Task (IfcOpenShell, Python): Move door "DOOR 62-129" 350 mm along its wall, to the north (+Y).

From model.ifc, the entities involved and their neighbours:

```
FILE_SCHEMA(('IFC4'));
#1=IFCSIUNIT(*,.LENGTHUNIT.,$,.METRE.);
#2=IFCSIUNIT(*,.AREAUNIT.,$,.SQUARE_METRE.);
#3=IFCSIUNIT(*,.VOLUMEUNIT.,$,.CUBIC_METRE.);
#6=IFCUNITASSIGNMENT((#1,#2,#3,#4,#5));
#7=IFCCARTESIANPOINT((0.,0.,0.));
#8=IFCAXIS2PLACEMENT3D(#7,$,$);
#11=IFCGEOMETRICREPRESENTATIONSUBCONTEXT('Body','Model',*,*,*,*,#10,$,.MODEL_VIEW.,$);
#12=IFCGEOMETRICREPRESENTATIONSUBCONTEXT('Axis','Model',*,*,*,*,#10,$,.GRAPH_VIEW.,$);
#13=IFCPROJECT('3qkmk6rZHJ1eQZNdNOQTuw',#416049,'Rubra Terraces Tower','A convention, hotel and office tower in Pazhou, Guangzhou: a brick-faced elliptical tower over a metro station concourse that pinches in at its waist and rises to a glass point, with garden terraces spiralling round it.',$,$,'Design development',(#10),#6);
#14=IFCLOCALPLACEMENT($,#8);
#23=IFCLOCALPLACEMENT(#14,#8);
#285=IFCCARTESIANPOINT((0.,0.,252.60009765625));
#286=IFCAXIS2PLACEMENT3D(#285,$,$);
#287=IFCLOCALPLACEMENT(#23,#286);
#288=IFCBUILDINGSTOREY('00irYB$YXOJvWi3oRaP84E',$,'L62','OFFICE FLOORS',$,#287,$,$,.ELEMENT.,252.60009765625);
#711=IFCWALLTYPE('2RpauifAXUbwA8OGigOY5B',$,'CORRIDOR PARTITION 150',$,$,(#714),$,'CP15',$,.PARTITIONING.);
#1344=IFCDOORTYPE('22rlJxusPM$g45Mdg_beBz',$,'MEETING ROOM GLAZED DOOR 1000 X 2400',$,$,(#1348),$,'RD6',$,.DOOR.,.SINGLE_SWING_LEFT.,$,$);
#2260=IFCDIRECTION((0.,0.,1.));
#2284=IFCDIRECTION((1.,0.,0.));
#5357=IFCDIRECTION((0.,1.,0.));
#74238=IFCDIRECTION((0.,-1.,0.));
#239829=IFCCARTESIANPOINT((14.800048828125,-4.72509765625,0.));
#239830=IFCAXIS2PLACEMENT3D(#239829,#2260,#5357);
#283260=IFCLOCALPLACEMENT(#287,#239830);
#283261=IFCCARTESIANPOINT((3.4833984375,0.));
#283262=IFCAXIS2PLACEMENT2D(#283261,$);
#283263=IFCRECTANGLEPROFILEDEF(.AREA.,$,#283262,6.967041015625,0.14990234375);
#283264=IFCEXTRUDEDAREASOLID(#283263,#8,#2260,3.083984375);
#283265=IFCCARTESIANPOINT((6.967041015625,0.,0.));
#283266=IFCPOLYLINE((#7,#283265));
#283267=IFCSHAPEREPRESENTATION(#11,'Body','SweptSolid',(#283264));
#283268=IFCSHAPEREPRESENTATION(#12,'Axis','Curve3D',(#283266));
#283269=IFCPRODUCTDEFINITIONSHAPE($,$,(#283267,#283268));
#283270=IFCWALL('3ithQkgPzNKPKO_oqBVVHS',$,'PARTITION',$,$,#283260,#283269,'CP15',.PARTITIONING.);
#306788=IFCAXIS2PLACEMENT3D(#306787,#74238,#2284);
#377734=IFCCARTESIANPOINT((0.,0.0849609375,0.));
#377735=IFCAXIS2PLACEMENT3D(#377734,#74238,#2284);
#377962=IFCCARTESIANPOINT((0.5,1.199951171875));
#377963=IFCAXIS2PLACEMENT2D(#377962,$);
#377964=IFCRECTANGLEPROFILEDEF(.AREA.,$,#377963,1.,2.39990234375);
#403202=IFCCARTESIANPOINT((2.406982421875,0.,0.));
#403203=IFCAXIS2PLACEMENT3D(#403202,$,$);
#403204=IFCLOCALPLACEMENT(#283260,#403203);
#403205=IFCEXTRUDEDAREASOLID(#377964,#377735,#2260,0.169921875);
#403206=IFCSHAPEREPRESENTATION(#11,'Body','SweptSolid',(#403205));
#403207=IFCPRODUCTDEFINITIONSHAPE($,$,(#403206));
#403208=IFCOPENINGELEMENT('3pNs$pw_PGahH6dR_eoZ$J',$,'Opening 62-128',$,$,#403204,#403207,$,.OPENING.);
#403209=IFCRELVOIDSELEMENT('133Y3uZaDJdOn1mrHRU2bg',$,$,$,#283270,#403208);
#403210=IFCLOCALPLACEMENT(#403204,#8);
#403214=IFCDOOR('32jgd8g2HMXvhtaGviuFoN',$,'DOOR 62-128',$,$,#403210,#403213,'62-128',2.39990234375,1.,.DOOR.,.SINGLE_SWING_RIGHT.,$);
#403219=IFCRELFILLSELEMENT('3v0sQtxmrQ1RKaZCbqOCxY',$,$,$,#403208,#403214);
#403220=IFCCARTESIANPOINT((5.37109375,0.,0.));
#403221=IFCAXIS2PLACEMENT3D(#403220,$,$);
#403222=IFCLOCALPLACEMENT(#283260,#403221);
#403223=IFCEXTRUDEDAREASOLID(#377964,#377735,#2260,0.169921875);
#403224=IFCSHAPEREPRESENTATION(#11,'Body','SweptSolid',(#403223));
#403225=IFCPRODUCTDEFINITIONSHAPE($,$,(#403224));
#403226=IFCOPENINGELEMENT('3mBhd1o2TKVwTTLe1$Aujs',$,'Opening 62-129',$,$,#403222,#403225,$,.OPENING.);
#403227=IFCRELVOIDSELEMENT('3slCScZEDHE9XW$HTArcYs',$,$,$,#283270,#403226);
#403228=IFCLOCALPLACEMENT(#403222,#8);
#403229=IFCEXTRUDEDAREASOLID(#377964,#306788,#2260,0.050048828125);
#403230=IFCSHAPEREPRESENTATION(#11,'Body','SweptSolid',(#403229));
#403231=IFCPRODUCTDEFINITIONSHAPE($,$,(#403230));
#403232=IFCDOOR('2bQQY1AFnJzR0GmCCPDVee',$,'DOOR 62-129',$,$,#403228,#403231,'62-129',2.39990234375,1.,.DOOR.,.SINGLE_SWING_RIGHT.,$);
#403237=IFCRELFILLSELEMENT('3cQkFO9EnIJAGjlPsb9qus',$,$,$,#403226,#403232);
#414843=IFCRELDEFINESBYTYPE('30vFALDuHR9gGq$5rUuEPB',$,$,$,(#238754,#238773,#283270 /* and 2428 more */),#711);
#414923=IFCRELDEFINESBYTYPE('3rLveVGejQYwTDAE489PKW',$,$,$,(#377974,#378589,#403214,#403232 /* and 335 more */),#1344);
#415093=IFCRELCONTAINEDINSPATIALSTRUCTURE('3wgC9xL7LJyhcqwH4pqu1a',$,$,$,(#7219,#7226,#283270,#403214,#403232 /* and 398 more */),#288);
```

```python
import ifcopenshell
import ifcopenshell.api.geometry
import ifcopenshell.util.placement

model = ifcopenshell.open("model.ifc")

door = model.by_guid("2bQQY1AFnJzR0GmCCPDVee")
opening = door.FillsVoids[0].RelatingOpeningElement
wall = opening.VoidsElements[0].RelatingBuildingElement

wall_matrix = ifcopenshell.util.placement.get_local_placement(wall.ObjectPlacement)
shift = wall_matrix[:3, 0] * 0.35
before = ifcopenshell.util.placement.get_local_placement(door.ObjectPlacement)[:3, 3].copy()

# The door is placed relative to its opening, so it follows when the opening moves.
matrix = ifcopenshell.util.placement.get_local_placement(opening.ObjectPlacement)
matrix[:3, 3] += shift
ifcopenshell.api.geometry.edit_object_placement(
    model, product=opening, matrix=matrix, is_si=False, should_transform_children=True
)

after = ifcopenshell.util.placement.get_local_placement(door.ObjectPlacement)[:3, 3]
print("door moved by", (after - before).round(3) + 0.0)

model.write("model-out.ifc")
```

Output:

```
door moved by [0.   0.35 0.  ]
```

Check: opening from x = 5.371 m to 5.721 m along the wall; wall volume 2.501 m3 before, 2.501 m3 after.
